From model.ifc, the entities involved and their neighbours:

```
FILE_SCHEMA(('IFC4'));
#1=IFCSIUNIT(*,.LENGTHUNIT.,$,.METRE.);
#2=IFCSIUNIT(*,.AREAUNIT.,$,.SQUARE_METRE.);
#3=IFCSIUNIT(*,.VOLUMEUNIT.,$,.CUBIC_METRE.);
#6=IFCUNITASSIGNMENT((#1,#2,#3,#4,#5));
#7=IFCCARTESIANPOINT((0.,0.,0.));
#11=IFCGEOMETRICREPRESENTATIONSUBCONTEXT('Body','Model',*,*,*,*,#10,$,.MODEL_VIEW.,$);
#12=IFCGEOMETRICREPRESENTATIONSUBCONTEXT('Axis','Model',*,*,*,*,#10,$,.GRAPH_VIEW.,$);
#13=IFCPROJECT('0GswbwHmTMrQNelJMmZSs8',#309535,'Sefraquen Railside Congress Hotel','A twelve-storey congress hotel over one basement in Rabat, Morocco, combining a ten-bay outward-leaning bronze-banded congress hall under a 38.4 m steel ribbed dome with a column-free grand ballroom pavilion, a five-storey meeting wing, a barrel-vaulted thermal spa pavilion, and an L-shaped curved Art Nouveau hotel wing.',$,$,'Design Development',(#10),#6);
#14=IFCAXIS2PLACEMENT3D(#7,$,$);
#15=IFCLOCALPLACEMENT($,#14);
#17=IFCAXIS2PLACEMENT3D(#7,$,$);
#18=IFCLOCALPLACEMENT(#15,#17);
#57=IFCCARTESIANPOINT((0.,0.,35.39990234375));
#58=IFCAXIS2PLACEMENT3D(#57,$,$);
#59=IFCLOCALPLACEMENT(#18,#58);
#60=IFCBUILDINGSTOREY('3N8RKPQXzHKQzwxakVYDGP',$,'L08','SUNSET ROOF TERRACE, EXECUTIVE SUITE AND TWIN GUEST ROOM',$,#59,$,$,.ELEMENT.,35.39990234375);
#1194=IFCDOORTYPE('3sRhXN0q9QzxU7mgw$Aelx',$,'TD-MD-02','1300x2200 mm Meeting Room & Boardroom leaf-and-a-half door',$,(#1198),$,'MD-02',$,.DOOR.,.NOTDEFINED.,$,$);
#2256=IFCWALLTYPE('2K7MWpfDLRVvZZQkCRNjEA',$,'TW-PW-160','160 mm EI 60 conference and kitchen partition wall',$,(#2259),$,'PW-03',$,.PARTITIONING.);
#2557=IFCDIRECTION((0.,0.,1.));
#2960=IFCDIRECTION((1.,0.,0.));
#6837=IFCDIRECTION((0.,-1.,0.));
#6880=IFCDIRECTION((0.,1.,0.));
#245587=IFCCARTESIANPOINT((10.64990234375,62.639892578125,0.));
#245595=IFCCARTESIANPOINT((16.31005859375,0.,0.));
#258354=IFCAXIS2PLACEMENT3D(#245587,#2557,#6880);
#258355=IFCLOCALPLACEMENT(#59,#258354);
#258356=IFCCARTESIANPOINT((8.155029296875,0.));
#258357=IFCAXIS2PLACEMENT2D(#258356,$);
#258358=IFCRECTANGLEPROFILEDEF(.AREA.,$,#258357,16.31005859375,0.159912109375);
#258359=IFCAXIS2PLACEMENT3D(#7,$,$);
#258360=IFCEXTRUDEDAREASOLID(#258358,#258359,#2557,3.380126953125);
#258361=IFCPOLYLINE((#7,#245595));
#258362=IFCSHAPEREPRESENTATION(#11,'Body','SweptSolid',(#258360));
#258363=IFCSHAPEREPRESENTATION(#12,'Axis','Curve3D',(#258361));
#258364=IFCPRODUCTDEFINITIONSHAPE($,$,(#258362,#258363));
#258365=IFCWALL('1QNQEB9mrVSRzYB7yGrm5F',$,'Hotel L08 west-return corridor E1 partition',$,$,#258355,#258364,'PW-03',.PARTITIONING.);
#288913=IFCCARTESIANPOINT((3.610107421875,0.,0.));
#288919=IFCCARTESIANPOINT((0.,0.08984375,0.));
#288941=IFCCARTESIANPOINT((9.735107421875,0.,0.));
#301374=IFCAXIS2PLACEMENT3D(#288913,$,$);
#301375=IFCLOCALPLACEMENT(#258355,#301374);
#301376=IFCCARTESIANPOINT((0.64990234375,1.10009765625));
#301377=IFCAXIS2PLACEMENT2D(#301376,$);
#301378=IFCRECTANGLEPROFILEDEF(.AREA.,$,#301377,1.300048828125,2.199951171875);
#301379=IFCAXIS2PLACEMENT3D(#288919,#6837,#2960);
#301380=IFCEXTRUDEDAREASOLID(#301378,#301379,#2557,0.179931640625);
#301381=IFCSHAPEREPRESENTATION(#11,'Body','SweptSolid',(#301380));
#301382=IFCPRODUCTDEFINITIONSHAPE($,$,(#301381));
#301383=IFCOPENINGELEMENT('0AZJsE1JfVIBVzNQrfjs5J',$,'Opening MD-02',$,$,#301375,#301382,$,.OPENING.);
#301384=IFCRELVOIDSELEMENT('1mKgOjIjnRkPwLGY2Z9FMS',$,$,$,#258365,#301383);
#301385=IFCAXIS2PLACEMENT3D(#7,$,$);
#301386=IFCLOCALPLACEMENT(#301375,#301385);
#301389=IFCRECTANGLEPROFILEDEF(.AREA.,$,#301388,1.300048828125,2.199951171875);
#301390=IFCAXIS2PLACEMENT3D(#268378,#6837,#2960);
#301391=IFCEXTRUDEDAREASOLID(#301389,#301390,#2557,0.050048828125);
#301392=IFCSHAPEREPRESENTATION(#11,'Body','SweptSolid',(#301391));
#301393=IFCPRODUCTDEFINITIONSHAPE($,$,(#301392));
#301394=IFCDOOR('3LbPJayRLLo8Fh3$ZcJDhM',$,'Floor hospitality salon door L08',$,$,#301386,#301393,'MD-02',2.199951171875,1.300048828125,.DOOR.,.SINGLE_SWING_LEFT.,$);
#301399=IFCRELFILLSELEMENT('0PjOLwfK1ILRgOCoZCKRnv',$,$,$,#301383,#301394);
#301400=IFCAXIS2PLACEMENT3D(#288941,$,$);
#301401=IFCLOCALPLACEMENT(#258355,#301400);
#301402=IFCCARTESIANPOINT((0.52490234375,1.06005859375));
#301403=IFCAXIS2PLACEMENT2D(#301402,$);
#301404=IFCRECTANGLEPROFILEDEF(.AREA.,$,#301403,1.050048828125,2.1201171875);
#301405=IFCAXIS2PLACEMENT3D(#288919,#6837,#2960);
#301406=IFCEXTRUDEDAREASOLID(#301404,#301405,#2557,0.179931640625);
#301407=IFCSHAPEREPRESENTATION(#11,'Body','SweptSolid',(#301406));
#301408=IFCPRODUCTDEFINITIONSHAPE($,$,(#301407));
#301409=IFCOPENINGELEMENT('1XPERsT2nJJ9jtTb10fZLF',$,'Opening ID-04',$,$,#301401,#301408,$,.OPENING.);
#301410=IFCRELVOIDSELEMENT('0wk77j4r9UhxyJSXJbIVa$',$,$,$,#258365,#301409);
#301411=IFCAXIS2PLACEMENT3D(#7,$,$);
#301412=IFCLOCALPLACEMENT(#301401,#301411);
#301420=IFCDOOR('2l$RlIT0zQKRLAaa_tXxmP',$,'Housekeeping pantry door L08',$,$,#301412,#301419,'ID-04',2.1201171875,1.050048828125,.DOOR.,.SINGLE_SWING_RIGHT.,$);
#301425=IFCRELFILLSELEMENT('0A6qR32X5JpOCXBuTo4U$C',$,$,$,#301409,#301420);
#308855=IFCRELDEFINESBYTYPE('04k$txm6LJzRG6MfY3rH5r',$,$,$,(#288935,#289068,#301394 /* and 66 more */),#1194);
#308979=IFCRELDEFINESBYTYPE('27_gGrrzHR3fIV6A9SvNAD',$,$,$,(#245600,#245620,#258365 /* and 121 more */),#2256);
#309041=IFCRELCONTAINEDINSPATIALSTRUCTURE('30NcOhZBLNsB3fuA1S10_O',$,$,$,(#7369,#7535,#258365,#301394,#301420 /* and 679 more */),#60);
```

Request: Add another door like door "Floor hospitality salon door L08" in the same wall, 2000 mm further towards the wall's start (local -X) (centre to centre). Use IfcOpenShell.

```python
import ifcopenshell
import ifcopenshell.api.feature
import ifcopenshell.api.geometry
import ifcopenshell.api.root
import ifcopenshell.geom
import ifcopenshell.util.element
import ifcopenshell.util.placement
import ifcopenshell.util.shape
import ifcopenshell.util.unit

model = ifcopenshell.open("model.ifc")
unit_scale = ifcopenshell.util.unit.calculate_unit_scale(model)
settings = ifcopenshell.geom.settings()


def volume(element):
    """Net volume in cubic metres, openings subtracted."""
    shape = ifcopenshell.geom.create_shape(settings, element)
    return ifcopenshell.util.shape.get_volume(shape.geometry)


door = model.by_guid("3LbPJayRLLo8Fh3$ZcJDhM")
opening = door.FillsVoids[0].RelatingOpeningElement
wall = opening.VoidsElements[0].RelatingBuildingElement
before = volume(wall)
shift = ifcopenshell.util.placement.get_local_placement(wall.ObjectPlacement)[:3, 0] * -2 / unit_scale

# copy_class copies the void relationship, type, container and properties, but no geometry.
new_opening = ifcopenshell.api.root.copy_class(model, product=opening)
new_opening.Representation = ifcopenshell.util.element.copy_deep(
    model, opening.Representation, exclude=["IfcGeometricRepresentationContext", "IfcRepresentationMap"]
)
new_door = ifcopenshell.api.root.copy_class(model, product=door)
new_door.Representation = ifcopenshell.util.element.copy_deep(
    model, door.Representation, exclude=["IfcGeometricRepresentationContext", "IfcRepresentationMap"]
)
new_door.Tag = None
ifcopenshell.api.feature.add_filling(model, opening=new_opening, element=new_door)

for old, new in ((opening, new_opening), (door, new_door)):
    matrix = ifcopenshell.util.placement.get_local_placement(old.ObjectPlacement)
    matrix[:3, 3] += shift
    ifcopenshell.api.geometry.edit_object_placement(model, product=new, matrix=matrix, is_si=False)

after = volume(wall)

print(f"wall volume {before:.3f} -> {after:.3f} m3")

model.write("model_v2.ifc")
```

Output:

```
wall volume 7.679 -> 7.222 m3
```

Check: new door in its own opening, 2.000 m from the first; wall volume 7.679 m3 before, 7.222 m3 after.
